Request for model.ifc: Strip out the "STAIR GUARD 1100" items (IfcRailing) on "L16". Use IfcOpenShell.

First a look at what the model holds.

```python
import ifcopenshell
import ifcopenshell.util.element

model = ifcopenshell.open("model.ifc")
print(model.schema)
storey = next(s for s in model.by_type("IfcBuildingStorey") if s.Name == "L16")
railings = [e for e in ifcopenshell.util.element.get_decomposition(storey) if e.is_a("IfcRailing")]
seen = {}
for e in railings:
    element_type = ifcopenshell.util.element.get_type(e)
    name = element_type.Name if element_type not in (None, e) else None
    seen[name] = seen.get(name, 0) + 1
for name, count in sorted(seen.items(), key=str):
    print(count, "x", name)
```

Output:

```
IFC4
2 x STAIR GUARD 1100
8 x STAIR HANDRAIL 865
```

```python
import ifcopenshell
import ifcopenshell.api.root
import ifcopenshell.util.element

model = ifcopenshell.open("model.ifc")

storey = next(s for s in model.by_type("IfcBuildingStorey") if s.Name == "L16")
railings = [e for e in ifcopenshell.util.element.get_decomposition(storey) if e.is_a("IfcRailing")]
targets = [e for e in railings if (t := ifcopenshell.util.element.get_type(e)) not in (None, e) and t.Name == "STAIR GUARD 1100"]

for e in targets:
    ifcopenshell.api.root.remove_product(model, product=e)
print(len(targets), "removed")

model.write("model_rev.ifc")
```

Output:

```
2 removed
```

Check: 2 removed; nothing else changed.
